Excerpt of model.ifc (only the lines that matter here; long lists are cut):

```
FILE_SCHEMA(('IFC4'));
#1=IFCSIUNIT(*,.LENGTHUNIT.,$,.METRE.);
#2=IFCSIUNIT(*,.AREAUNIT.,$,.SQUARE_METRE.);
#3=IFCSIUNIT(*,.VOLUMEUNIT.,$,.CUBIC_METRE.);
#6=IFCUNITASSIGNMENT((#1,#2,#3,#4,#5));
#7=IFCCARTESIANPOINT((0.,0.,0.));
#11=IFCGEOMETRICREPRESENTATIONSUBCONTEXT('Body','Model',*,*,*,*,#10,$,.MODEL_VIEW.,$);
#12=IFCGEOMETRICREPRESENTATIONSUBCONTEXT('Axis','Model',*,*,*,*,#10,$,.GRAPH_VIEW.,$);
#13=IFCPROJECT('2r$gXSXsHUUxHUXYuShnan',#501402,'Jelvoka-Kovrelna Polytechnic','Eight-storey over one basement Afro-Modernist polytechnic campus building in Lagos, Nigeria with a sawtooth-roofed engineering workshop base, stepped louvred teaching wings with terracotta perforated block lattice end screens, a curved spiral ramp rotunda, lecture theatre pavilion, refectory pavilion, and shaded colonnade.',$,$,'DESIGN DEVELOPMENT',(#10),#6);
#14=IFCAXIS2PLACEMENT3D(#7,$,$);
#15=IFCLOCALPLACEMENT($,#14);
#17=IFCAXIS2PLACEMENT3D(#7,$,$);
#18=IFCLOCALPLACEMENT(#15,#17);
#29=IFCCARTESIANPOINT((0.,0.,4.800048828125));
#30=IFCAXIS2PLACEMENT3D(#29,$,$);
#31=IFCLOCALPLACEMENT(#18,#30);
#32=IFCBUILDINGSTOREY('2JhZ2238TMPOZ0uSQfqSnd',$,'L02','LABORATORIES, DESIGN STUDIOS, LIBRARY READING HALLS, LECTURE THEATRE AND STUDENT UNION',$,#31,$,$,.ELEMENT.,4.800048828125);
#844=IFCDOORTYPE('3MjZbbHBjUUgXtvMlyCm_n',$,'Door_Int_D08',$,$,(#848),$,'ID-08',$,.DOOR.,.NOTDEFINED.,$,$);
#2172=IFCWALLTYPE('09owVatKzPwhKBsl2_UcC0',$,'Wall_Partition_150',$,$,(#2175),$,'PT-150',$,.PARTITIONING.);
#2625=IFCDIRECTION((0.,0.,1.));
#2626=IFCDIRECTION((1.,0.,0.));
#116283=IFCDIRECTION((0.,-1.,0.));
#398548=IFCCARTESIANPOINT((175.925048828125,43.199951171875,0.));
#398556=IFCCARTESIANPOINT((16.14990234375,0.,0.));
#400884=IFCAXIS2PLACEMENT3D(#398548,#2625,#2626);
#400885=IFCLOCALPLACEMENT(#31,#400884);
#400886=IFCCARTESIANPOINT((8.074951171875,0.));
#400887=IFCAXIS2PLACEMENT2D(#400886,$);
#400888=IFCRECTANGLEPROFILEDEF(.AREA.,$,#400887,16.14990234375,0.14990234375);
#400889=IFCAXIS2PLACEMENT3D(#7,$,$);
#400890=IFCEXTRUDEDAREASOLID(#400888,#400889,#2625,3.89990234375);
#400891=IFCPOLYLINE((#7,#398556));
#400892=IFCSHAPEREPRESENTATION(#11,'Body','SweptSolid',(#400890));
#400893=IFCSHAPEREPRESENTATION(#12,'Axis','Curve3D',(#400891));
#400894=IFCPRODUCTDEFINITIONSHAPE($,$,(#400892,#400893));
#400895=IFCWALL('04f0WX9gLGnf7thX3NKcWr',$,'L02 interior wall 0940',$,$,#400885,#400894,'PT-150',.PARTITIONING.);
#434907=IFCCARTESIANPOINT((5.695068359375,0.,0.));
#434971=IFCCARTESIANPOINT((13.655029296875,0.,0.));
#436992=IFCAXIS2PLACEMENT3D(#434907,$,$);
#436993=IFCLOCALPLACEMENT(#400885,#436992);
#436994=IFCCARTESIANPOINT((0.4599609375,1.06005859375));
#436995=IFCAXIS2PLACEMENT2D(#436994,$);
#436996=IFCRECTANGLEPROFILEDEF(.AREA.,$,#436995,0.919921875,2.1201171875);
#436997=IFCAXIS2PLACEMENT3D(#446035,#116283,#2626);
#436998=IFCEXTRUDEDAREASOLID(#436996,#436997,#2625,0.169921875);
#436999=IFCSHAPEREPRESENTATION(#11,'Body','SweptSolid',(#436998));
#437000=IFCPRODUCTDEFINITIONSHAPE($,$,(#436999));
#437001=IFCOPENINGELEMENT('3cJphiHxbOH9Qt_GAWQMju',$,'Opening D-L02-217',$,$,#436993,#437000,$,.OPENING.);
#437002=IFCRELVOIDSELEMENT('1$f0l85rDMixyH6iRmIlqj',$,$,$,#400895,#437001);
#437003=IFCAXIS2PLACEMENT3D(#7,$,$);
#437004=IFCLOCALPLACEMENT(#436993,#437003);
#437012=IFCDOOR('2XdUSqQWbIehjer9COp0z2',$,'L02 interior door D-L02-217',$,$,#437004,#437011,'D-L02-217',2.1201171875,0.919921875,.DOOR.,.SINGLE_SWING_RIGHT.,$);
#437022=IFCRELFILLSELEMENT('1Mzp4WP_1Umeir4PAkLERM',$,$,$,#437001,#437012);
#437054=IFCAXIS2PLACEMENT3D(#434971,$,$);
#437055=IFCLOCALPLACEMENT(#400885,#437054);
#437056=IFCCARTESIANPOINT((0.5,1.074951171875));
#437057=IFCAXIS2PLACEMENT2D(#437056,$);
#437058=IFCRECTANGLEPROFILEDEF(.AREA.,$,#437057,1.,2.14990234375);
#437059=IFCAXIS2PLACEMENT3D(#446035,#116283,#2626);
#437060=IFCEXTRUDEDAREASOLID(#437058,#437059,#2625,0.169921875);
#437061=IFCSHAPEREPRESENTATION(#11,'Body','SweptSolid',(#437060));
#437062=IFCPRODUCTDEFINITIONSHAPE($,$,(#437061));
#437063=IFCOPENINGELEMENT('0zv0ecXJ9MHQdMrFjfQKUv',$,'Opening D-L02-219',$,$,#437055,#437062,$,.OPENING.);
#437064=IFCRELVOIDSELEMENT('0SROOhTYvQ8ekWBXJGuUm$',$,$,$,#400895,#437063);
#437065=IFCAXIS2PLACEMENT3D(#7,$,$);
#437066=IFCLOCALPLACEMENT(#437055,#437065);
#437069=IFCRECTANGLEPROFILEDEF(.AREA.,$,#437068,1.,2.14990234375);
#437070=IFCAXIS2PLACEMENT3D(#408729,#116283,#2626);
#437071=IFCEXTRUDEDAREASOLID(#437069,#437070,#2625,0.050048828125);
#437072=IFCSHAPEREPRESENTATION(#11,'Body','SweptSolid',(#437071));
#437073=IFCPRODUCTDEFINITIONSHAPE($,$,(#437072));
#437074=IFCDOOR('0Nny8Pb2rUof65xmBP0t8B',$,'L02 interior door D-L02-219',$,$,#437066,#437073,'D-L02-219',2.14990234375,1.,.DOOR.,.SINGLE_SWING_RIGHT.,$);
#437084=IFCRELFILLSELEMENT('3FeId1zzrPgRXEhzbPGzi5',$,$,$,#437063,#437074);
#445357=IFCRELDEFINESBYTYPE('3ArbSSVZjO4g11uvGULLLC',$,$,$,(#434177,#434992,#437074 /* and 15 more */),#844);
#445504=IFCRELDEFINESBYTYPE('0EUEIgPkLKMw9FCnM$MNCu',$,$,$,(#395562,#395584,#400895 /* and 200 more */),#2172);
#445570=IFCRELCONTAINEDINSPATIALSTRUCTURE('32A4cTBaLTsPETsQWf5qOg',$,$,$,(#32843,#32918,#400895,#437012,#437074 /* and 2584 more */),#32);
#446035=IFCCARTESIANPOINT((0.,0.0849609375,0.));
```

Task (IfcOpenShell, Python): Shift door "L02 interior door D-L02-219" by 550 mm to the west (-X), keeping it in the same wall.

```python
import ifcopenshell
import ifcopenshell.api.geometry
import ifcopenshell.util.placement

model = ifcopenshell.open("model.ifc")

door = model.by_id(437074)
opening = door.FillsVoids[0].RelatingOpeningElement
wall = opening.VoidsElements[0].RelatingBuildingElement

wall_matrix = ifcopenshell.util.placement.get_local_placement(wall.ObjectPlacement)
shift = wall_matrix[:3, 0] * -0.55
before = ifcopenshell.util.placement.get_local_placement(door.ObjectPlacement)[:3, 3].copy()

# The door is placed relative to its opening, so it follows when the opening moves.
matrix = ifcopenshell.util.placement.get_local_placement(opening.ObjectPlacement)
matrix[:3, 3] += shift
ifcopenshell.api.geometry.edit_object_placement(
    model, product=opening, matrix=matrix, is_si=False, should_transform_children=True
)

after = ifcopenshell.util.placement.get_local_placement(door.ObjectPlacement)[:3, 3]
print("door moved by", (after - before).round(3) + 0.0)

model.write("model_edited.ifc")
```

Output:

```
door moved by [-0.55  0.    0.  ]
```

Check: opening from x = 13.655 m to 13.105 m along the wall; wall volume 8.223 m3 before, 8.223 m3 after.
